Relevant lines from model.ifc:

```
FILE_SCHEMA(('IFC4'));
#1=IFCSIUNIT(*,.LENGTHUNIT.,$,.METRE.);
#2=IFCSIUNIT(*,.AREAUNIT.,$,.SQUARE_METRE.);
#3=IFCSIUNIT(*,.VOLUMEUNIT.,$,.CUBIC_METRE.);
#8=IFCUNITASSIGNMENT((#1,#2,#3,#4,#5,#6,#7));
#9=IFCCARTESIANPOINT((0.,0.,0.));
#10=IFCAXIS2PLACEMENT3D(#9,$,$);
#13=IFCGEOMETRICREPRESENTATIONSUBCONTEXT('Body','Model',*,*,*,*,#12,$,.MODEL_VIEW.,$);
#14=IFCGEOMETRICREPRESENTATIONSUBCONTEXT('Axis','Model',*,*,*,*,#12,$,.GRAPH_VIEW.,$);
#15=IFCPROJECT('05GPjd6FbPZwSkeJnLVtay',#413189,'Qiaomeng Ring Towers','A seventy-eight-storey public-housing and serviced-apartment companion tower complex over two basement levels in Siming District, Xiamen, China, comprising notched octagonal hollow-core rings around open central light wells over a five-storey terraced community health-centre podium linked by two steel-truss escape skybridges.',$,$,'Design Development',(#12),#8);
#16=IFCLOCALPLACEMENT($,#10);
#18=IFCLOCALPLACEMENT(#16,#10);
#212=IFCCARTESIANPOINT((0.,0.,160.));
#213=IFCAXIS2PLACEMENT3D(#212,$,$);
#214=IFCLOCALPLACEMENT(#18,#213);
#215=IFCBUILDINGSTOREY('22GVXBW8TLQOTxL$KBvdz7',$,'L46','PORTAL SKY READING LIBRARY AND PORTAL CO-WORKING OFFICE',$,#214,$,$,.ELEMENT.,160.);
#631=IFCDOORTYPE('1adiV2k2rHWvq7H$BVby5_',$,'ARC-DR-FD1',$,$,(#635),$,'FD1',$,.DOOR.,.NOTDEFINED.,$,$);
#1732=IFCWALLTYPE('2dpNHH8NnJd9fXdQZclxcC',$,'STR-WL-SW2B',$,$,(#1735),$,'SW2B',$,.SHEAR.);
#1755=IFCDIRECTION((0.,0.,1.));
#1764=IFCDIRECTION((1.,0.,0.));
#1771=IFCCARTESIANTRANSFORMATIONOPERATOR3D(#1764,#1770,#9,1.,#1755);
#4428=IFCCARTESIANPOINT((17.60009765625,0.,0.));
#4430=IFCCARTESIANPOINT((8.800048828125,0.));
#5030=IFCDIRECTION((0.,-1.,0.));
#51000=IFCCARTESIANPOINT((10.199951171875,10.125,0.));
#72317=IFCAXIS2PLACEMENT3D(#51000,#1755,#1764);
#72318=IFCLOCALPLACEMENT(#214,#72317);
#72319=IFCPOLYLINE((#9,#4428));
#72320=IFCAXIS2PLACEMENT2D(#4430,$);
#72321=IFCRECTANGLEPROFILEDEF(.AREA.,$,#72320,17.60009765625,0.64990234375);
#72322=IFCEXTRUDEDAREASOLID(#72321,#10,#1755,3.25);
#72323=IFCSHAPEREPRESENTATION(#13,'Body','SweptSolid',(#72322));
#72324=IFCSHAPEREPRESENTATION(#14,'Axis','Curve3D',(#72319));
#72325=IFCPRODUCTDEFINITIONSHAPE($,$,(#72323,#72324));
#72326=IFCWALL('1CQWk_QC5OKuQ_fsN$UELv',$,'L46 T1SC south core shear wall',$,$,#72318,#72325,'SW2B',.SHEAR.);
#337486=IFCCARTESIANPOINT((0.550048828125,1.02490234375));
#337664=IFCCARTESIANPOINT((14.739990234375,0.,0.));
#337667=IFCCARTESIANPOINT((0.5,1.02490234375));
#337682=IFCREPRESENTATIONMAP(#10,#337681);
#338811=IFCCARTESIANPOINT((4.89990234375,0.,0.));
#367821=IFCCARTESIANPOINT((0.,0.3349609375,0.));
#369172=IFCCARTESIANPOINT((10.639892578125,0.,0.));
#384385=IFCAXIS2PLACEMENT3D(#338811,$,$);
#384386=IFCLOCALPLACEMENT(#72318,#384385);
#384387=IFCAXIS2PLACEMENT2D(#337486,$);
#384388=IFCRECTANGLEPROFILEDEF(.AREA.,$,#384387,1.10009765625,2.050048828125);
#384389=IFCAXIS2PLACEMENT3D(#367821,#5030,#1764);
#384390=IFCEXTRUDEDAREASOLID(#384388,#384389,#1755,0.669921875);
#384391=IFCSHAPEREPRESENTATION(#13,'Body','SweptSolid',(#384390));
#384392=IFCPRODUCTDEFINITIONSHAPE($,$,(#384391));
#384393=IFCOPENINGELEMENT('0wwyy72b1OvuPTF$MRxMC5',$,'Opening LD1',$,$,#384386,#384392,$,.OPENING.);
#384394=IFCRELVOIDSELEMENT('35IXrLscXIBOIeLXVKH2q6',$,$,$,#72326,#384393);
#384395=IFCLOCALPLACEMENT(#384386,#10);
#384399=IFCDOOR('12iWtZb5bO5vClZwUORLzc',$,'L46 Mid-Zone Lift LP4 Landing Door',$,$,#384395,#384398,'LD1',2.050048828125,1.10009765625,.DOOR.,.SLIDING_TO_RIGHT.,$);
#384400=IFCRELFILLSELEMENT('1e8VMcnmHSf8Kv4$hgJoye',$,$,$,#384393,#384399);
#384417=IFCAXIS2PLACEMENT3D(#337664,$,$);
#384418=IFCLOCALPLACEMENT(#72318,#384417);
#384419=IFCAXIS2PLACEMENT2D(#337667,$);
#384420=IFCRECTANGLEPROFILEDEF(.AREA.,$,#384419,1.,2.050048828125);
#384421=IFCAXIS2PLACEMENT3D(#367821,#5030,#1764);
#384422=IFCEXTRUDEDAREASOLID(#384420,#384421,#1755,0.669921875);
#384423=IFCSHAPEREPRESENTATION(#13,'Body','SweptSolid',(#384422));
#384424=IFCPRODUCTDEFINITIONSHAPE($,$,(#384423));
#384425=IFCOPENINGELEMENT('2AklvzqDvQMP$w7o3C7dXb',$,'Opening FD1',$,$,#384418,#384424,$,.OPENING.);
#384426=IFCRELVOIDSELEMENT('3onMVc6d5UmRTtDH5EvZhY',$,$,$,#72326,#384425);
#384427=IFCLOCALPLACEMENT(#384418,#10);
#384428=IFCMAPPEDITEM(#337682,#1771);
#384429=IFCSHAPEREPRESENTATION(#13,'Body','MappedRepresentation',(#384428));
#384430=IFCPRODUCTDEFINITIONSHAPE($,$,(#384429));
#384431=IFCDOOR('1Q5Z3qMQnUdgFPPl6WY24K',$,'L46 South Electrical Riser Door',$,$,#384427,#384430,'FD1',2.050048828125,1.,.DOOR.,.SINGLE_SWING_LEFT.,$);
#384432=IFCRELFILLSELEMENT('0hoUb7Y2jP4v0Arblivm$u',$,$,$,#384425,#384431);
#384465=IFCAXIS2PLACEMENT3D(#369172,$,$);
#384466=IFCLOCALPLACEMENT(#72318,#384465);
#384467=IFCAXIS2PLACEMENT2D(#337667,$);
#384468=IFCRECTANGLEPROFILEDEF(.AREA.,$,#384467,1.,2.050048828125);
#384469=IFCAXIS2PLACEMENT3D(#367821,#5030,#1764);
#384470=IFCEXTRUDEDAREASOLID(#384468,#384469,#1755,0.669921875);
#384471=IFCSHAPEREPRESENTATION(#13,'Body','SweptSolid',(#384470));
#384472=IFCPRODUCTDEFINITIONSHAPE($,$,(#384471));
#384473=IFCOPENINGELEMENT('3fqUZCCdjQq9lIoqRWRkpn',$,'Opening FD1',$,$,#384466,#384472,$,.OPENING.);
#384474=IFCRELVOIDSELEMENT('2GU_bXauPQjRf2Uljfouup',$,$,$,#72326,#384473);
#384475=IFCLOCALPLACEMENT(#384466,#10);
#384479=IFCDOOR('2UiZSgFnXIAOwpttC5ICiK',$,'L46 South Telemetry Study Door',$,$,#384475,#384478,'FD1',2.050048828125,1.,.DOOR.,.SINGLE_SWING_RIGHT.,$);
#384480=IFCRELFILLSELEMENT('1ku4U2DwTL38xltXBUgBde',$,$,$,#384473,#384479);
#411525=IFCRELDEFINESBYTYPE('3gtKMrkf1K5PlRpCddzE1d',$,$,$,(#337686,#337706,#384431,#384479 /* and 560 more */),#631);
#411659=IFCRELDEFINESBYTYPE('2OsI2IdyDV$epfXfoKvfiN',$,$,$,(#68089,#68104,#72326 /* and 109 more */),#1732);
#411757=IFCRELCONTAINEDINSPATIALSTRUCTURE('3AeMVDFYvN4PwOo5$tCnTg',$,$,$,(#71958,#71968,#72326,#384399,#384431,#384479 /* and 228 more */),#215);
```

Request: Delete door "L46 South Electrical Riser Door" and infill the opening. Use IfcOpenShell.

```python
import ifcopenshell
import ifcopenshell.api.feature
import ifcopenshell.api.root
import ifcopenshell.geom
import ifcopenshell.util.shape

model = ifcopenshell.open("model.ifc")
settings = ifcopenshell.geom.settings()


def volume(element):
    """Net volume in cubic metres, openings subtracted."""
    shape = ifcopenshell.geom.create_shape(settings, element)
    return ifcopenshell.util.shape.get_volume(shape.geometry)


door = model.by_id(384431)
opening = door.FillsVoids[0].RelatingOpeningElement
wall = opening.VoidsElements[0].RelatingBuildingElement
before = volume(wall)

ifcopenshell.api.root.remove_product(model, product=door)
ifcopenshell.api.feature.remove_feature(model, feature=opening)

after = volume(wall)

print(f"wall volume {before:.3f} -> {after:.3f} m3")

model.write("model_updated.ifc")
```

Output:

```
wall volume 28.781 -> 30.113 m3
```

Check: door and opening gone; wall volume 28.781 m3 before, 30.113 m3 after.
